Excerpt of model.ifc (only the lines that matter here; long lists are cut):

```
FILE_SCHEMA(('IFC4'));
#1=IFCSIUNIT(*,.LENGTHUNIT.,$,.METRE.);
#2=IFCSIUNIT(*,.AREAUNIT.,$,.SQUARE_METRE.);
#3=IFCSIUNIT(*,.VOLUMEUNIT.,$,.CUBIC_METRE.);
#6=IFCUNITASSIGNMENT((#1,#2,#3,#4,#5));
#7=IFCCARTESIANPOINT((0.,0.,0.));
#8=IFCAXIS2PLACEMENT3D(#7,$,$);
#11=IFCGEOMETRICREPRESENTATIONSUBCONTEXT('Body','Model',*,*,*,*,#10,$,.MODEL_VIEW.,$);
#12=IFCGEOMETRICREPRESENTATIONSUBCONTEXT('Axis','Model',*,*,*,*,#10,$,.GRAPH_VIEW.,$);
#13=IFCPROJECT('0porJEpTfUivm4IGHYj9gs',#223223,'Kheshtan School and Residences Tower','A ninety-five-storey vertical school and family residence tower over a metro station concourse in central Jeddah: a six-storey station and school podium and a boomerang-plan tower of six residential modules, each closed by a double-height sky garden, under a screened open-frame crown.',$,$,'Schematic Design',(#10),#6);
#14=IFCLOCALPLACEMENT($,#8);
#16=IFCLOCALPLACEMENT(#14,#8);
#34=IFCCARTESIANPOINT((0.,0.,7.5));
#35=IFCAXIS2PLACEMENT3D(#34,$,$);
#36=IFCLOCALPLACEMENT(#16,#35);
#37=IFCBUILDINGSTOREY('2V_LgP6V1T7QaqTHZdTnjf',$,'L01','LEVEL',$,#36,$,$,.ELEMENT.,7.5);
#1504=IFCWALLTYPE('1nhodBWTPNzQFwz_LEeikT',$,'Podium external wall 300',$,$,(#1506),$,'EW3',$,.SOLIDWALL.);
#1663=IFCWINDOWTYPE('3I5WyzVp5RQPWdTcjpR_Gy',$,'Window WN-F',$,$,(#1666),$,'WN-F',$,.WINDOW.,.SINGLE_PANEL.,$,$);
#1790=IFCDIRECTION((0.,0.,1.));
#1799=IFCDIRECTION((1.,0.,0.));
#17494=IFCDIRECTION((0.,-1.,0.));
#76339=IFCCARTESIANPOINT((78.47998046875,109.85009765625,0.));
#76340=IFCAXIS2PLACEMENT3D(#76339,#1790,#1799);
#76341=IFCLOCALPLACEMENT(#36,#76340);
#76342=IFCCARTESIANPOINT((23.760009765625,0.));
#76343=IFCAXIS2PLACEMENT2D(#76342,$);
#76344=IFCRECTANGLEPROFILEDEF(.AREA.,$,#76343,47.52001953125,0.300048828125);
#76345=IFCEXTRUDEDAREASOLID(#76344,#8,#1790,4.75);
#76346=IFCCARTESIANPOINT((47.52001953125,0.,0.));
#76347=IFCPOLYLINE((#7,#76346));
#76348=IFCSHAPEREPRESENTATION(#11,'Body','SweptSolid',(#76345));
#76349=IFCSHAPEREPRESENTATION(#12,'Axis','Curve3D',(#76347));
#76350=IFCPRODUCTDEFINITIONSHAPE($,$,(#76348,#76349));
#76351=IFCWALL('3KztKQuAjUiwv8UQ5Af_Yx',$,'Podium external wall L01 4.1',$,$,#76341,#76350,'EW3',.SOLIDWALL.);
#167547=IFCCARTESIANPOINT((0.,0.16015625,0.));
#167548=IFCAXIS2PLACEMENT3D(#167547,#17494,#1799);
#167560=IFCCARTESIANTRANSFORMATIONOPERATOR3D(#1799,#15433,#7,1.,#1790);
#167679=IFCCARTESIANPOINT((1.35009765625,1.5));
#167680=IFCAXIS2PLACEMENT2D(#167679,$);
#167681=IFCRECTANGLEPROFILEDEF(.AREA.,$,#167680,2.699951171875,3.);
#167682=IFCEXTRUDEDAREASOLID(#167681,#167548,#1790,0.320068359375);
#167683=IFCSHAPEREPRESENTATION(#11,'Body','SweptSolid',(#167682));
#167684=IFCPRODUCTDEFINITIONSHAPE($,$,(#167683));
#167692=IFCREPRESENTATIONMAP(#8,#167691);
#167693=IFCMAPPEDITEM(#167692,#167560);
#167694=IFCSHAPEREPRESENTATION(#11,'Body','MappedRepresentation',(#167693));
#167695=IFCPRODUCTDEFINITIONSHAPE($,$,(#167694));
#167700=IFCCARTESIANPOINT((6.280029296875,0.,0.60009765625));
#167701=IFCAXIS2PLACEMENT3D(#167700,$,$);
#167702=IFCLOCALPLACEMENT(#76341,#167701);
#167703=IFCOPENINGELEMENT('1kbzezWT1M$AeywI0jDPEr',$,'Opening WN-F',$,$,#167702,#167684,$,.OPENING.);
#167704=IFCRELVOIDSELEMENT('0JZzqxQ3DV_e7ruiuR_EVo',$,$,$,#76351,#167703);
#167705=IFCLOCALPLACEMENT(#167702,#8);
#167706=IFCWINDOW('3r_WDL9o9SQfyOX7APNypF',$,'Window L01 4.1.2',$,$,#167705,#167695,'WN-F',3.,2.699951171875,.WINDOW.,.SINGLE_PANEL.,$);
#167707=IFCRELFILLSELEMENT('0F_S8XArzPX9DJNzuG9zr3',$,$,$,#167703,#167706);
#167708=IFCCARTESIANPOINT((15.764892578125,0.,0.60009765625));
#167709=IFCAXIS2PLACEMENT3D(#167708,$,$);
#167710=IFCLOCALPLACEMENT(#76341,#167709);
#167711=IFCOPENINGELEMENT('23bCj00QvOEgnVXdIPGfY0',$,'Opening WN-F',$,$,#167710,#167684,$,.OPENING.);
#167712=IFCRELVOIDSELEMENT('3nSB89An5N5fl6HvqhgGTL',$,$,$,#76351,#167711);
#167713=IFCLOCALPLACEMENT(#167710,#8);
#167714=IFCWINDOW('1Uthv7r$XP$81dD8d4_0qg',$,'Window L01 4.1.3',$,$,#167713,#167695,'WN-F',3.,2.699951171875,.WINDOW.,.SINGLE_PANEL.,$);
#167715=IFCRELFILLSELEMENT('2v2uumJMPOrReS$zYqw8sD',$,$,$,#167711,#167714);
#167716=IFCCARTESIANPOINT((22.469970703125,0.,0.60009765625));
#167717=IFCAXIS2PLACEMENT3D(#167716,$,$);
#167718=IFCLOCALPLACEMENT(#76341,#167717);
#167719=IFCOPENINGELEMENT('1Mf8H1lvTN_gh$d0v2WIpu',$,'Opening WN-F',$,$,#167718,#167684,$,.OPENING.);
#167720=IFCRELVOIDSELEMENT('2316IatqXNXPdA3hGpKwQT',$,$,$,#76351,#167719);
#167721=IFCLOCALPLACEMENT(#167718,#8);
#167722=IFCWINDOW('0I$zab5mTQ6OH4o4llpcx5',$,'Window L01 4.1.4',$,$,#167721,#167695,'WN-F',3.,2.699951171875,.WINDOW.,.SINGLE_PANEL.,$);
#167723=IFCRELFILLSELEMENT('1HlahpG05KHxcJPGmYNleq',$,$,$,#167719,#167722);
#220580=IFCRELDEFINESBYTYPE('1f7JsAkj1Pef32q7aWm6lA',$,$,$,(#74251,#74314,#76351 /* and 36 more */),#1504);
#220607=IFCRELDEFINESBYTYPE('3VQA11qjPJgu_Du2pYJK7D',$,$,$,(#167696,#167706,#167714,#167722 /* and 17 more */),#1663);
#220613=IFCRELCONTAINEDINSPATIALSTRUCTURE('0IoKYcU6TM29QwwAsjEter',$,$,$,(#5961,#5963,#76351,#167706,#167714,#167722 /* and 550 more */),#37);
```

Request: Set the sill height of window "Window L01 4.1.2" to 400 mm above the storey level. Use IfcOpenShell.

```python
import numpy as np
import ifcopenshell
import ifcopenshell.api.geometry
import ifcopenshell.geom
import ifcopenshell.util.element
import ifcopenshell.util.placement
import ifcopenshell.util.shape
import ifcopenshell.util.unit

model = ifcopenshell.open("model.ifc")
unit_scale = ifcopenshell.util.unit.calculate_unit_scale(model)

window = model.by_guid("3r_WDL9o9SQfyOX7APNypF")
opening = window.FillsVoids[0].RelatingOpeningElement
storey = ifcopenshell.util.element.get_container(window, ifc_class="IfcBuildingStorey")
level = ifcopenshell.util.placement.get_local_placement(storey.ObjectPlacement)[2, 3]

# The opening's origin need not be at the sill, so measure its lowest point.
shape = ifcopenshell.geom.create_shape(ifcopenshell.geom.settings(), opening)
bottom = ifcopenshell.util.shape.get_shape_bottom_elevation(shape, shape.geometry) / unit_scale
dz = level + 0.4 / unit_scale - bottom

shift = np.array([0.0, 0.0, dz])
# The window is placed relative to its opening, so it follows when the opening moves.
matrix = ifcopenshell.util.placement.get_local_placement(opening.ObjectPlacement)
matrix[:3, 3] += shift
ifcopenshell.api.geometry.edit_object_placement(
    model, product=opening, matrix=matrix, is_si=False, should_transform_children=True
)

print(f"moved by {dz * unit_scale:+.3f} m")

model.write("model_rev.ifc")
```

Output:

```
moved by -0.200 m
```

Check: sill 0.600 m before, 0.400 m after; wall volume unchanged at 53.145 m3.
